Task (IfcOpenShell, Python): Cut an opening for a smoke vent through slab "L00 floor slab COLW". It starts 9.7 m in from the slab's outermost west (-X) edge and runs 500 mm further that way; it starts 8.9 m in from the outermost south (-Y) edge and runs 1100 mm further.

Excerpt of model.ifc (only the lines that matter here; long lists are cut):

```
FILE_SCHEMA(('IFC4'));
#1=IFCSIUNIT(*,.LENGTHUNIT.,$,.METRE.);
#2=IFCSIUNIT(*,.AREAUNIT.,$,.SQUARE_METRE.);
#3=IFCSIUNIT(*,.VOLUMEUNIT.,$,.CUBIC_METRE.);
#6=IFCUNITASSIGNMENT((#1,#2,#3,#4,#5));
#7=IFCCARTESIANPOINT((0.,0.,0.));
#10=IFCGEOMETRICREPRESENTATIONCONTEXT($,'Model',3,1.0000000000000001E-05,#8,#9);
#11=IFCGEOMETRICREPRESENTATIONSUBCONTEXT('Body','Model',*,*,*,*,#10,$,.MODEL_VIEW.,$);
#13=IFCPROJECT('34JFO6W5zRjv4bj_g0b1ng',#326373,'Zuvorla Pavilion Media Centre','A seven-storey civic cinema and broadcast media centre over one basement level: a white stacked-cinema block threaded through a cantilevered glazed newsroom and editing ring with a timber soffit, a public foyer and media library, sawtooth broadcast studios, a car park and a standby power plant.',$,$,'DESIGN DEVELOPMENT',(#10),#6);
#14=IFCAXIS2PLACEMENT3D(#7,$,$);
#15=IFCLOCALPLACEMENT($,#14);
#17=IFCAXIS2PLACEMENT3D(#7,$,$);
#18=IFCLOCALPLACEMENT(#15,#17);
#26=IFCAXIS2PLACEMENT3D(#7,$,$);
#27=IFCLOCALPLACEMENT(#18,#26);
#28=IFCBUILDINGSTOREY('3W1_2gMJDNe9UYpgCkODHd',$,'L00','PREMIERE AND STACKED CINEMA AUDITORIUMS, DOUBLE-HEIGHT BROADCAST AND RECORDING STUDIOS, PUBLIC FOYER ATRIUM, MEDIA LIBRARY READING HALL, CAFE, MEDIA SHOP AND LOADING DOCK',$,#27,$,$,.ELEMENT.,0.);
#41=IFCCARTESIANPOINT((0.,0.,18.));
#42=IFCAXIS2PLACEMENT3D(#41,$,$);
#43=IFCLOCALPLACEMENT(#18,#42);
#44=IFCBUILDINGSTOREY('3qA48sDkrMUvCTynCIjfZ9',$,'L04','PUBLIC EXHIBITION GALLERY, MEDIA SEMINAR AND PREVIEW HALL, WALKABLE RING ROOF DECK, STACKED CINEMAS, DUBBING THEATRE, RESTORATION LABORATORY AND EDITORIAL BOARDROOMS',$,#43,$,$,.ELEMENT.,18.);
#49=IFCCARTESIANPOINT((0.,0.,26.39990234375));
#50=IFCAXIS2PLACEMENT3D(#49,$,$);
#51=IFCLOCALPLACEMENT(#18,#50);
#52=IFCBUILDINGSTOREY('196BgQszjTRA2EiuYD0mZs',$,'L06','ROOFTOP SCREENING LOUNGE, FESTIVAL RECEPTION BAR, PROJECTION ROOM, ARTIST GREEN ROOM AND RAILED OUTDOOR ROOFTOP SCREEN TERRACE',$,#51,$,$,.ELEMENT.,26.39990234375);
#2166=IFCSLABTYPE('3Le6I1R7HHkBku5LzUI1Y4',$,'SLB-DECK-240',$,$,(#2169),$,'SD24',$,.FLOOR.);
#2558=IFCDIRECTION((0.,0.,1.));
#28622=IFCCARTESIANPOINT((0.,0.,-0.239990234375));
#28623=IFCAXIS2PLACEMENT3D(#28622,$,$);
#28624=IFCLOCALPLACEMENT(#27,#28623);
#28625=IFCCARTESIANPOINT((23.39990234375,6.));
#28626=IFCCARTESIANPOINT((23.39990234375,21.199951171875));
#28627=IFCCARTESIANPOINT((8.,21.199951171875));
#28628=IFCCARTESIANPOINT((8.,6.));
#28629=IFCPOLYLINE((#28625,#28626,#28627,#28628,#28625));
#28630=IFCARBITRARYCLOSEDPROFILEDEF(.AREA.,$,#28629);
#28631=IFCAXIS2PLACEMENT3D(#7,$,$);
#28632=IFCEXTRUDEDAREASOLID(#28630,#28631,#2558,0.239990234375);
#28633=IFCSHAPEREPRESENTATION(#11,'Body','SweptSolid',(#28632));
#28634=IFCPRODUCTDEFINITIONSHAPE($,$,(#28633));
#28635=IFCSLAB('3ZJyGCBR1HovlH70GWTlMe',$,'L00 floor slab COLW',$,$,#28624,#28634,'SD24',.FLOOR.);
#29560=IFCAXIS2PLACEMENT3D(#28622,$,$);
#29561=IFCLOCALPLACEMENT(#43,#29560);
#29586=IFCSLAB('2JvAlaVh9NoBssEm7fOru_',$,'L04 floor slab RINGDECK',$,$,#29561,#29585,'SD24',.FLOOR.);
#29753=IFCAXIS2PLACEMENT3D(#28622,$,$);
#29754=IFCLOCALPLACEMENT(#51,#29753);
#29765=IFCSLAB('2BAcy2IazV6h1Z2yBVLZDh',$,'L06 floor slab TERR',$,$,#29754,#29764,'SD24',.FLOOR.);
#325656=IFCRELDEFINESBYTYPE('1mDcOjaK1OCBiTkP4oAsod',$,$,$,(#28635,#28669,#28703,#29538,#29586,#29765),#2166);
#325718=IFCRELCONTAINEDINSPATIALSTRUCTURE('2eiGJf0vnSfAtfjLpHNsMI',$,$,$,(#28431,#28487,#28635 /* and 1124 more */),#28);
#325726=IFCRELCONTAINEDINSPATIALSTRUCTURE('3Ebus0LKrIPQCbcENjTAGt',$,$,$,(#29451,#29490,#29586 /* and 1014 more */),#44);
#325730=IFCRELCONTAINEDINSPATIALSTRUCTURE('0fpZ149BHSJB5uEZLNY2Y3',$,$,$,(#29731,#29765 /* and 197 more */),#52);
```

```python
import numpy as np
import ifcopenshell
import ifcopenshell.api.feature
import ifcopenshell.api.geometry
import ifcopenshell.api.root
import ifcopenshell.geom
import ifcopenshell.util.placement
import ifcopenshell.util.representation
import ifcopenshell.util.shape
import ifcopenshell.util.unit

model = ifcopenshell.open("model.ifc")
unit_scale = ifcopenshell.util.unit.calculate_unit_scale(model)
settings = ifcopenshell.geom.settings()


def volume(element):
    """Net volume in cubic metres, openings subtracted."""
    shape = ifcopenshell.geom.create_shape(settings, element)
    return ifcopenshell.util.shape.get_volume(shape.geometry)


slab = model.by_guid("3ZJyGCBR1HovlH70GWTlMe")
before = volume(slab)

# Extent in the slab's own axes, in metres. The edges named are its -X and -Y sides.
slab_shape = ifcopenshell.geom.create_shape(settings, slab)
vertices = ifcopenshell.util.shape.get_vertices(slab_shape.geometry)
x_min, y_min, bottom = vertices.min(axis=0)
top = vertices[:, 2].max()

opening = ifcopenshell.api.root.create_entity(model, ifc_class="IfcOpeningElement", name="Smoke vent opening", predefined_type="OPENING")
context = ifcopenshell.util.representation.get_context(model, "Model", "Body", "MODEL_VIEW")
width, depth = 0.5, 1.1
outline = [(0.0, 0.0), (width, 0.0), (width, depth), (0.0, depth), (0.0, 0.0)]
# Overshoot both faces by 50 mm so the cut is clean.
shape = ifcopenshell.api.geometry.add_slab_representation(
    model, context=context, depth=top - bottom + 0.1, polyline=outline
)
ifcopenshell.api.geometry.assign_representation(model, product=opening, representation=shape)

matrix = ifcopenshell.util.placement.get_local_placement(slab.ObjectPlacement)
matrix[:, 3] = matrix @ np.append(np.array([x_min + 9.7, y_min + 8.9, bottom - 0.05]) / unit_scale, 1.0)
ifcopenshell.api.geometry.edit_object_placement(model, product=opening, matrix=matrix, is_si=False)
ifcopenshell.api.feature.add_feature(model, feature=opening, element=slab)

after = volume(slab)

print(f"slab volume {before:.3f} -> {after:.3f} m3")

model.write("model_updated.ifc")
```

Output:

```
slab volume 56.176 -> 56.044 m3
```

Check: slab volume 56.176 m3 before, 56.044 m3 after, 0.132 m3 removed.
